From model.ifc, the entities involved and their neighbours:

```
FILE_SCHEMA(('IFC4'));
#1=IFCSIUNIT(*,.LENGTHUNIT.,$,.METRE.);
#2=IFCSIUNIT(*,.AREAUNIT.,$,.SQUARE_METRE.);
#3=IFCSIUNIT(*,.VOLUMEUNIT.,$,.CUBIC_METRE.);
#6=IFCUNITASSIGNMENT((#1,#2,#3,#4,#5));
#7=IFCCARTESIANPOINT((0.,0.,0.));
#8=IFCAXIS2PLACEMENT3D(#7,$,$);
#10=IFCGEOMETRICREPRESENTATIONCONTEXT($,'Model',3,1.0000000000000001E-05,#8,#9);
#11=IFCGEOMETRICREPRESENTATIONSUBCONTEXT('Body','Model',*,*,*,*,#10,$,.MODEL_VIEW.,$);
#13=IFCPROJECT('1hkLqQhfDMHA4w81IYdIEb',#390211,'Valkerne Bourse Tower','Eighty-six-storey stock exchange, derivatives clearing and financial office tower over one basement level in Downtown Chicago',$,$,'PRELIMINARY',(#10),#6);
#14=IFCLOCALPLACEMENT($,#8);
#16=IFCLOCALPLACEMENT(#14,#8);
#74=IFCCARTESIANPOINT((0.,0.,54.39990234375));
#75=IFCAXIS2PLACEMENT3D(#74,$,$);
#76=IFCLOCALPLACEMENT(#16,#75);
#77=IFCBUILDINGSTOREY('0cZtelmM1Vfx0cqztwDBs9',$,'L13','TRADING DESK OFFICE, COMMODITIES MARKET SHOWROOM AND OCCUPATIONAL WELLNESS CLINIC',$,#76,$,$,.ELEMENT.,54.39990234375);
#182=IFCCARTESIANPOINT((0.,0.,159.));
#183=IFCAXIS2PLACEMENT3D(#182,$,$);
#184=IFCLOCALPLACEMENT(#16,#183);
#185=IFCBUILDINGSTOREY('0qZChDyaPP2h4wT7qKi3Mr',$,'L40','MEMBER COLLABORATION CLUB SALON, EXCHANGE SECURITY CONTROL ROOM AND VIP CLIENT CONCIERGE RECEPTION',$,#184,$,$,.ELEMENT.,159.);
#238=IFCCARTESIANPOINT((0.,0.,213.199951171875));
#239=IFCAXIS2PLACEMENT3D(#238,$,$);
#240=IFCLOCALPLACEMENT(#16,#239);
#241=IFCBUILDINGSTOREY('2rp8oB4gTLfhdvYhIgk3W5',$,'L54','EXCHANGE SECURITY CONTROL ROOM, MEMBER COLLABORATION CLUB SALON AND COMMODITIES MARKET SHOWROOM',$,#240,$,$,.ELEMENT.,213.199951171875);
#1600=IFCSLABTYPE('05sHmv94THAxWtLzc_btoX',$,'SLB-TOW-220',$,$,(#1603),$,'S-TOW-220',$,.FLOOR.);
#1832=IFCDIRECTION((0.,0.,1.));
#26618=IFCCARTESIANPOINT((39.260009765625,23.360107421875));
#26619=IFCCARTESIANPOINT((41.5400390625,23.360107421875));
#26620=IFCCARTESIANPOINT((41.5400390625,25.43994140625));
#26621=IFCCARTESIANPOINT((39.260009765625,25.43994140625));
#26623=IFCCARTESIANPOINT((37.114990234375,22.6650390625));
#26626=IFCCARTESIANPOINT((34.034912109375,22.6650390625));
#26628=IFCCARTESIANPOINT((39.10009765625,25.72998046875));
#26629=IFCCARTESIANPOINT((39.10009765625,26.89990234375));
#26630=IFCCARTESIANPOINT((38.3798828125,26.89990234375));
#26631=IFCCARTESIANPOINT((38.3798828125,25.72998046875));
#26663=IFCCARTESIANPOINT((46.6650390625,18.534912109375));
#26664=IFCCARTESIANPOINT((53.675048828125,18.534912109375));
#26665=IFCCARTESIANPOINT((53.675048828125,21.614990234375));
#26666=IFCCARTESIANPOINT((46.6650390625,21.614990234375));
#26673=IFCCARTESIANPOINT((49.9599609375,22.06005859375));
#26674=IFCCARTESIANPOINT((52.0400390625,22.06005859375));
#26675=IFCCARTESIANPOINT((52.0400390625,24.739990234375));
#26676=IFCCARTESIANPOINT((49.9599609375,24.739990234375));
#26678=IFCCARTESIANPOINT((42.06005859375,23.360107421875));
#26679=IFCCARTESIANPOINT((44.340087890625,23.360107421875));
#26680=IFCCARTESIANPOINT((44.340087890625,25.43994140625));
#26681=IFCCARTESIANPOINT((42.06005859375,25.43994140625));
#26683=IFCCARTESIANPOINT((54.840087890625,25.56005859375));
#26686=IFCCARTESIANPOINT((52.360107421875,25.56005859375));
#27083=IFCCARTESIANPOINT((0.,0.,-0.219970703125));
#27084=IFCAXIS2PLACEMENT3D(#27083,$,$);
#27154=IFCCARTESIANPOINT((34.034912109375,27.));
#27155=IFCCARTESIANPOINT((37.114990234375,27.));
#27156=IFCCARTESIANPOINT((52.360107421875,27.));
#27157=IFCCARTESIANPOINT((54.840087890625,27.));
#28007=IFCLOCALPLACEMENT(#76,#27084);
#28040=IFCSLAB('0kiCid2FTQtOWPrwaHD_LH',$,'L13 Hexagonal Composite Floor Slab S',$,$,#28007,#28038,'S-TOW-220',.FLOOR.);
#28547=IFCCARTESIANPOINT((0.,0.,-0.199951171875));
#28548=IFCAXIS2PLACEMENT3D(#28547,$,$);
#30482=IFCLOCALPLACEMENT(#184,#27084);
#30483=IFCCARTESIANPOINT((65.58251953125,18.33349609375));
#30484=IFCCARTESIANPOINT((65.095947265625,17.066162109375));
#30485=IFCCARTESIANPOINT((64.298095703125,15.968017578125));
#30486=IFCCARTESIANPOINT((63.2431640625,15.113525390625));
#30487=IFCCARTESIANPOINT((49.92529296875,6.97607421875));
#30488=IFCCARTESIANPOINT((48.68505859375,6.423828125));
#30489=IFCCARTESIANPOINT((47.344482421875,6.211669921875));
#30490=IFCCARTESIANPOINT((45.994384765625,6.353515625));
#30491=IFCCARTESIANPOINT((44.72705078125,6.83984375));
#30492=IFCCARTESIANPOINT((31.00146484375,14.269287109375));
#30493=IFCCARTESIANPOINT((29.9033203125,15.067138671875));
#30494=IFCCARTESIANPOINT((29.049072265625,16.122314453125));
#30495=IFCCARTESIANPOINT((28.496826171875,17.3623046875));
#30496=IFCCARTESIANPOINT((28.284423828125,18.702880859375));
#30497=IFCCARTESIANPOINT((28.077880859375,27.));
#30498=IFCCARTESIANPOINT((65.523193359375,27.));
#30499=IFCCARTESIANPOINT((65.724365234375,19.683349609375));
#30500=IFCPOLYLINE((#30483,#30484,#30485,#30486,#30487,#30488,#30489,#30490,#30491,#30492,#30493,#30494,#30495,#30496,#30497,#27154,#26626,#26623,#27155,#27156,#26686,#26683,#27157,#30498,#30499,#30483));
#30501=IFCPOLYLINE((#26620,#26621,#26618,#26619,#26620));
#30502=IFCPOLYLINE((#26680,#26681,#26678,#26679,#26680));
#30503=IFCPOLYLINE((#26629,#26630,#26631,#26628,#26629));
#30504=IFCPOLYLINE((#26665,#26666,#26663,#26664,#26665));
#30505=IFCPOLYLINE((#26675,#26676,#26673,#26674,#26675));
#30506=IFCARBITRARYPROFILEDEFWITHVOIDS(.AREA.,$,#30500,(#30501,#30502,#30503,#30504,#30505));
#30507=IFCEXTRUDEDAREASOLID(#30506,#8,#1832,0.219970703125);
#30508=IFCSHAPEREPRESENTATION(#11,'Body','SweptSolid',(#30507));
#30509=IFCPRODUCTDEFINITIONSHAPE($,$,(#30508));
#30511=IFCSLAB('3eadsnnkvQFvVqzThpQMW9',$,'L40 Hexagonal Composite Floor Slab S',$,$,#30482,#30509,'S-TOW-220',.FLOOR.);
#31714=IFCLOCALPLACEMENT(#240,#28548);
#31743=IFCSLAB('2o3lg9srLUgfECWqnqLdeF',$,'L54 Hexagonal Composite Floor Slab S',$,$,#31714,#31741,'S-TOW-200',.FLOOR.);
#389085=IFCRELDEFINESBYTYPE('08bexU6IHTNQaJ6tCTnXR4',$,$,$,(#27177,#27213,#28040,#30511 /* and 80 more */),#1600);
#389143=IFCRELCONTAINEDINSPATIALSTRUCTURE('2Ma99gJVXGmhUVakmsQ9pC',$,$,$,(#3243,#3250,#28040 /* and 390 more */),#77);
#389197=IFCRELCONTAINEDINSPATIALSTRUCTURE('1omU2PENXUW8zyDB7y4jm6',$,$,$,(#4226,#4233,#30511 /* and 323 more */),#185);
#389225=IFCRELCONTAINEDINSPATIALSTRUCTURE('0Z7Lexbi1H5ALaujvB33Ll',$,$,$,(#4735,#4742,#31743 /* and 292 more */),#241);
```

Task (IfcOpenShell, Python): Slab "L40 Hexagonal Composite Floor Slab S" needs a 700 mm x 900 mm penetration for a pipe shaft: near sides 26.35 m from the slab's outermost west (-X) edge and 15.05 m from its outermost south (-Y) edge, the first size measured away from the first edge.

```python
import numpy as np
import ifcopenshell
import ifcopenshell.api.feature
import ifcopenshell.api.geometry
import ifcopenshell.api.root
import ifcopenshell.geom
import ifcopenshell.util.placement
import ifcopenshell.util.representation
import ifcopenshell.util.shape
import ifcopenshell.util.unit

model = ifcopenshell.open("model.ifc")
unit_scale = ifcopenshell.util.unit.calculate_unit_scale(model)
settings = ifcopenshell.geom.settings()


def volume(element):
    """Net volume in cubic metres, openings subtracted."""
    shape = ifcopenshell.geom.create_shape(settings, element)
    return ifcopenshell.util.shape.get_volume(shape.geometry)


slab = model.by_id(30511)
before = volume(slab)

# Extent in the slab's own axes, in metres. The edges named are its -X and -Y sides.
slab_shape = ifcopenshell.geom.create_shape(settings, slab)
vertices = ifcopenshell.util.shape.get_vertices(slab_shape.geometry)
x_min, y_min, bottom = vertices.min(axis=0)
top = vertices[:, 2].max()

opening = ifcopenshell.api.root.create_entity(model, ifc_class="IfcOpeningElement", name="Pipe shaft opening", predefined_type="OPENING")
context = ifcopenshell.util.representation.get_context(model, "Model", "Body", "MODEL_VIEW")
width, depth = 0.7, 0.9
outline = [(0.0, 0.0), (width, 0.0), (width, depth), (0.0, depth), (0.0, 0.0)]
# Overshoot both faces by 50 mm so the cut is clean.
shape = ifcopenshell.api.geometry.add_slab_representation(
    model, context=context, depth=top - bottom + 0.1, polyline=outline
)
ifcopenshell.api.geometry.assign_representation(model, product=opening, representation=shape)

matrix = ifcopenshell.util.placement.get_local_placement(slab.ObjectPlacement)
matrix[:, 3] = matrix @ np.append(np.array([x_min + 26.35, y_min + 15.05, bottom - 0.05]) / unit_scale, 1.0)
ifcopenshell.api.geometry.edit_object_placement(model, product=opening, matrix=matrix, is_si=False)
ifcopenshell.api.feature.add_feature(model, feature=opening, element=slab)

after = volume(slab)

print(f"slab volume {before:.3f} -> {after:.3f} m3")

model.write("model_v2.ifc")
```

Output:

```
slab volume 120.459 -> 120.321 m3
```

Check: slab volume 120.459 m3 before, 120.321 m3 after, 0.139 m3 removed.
